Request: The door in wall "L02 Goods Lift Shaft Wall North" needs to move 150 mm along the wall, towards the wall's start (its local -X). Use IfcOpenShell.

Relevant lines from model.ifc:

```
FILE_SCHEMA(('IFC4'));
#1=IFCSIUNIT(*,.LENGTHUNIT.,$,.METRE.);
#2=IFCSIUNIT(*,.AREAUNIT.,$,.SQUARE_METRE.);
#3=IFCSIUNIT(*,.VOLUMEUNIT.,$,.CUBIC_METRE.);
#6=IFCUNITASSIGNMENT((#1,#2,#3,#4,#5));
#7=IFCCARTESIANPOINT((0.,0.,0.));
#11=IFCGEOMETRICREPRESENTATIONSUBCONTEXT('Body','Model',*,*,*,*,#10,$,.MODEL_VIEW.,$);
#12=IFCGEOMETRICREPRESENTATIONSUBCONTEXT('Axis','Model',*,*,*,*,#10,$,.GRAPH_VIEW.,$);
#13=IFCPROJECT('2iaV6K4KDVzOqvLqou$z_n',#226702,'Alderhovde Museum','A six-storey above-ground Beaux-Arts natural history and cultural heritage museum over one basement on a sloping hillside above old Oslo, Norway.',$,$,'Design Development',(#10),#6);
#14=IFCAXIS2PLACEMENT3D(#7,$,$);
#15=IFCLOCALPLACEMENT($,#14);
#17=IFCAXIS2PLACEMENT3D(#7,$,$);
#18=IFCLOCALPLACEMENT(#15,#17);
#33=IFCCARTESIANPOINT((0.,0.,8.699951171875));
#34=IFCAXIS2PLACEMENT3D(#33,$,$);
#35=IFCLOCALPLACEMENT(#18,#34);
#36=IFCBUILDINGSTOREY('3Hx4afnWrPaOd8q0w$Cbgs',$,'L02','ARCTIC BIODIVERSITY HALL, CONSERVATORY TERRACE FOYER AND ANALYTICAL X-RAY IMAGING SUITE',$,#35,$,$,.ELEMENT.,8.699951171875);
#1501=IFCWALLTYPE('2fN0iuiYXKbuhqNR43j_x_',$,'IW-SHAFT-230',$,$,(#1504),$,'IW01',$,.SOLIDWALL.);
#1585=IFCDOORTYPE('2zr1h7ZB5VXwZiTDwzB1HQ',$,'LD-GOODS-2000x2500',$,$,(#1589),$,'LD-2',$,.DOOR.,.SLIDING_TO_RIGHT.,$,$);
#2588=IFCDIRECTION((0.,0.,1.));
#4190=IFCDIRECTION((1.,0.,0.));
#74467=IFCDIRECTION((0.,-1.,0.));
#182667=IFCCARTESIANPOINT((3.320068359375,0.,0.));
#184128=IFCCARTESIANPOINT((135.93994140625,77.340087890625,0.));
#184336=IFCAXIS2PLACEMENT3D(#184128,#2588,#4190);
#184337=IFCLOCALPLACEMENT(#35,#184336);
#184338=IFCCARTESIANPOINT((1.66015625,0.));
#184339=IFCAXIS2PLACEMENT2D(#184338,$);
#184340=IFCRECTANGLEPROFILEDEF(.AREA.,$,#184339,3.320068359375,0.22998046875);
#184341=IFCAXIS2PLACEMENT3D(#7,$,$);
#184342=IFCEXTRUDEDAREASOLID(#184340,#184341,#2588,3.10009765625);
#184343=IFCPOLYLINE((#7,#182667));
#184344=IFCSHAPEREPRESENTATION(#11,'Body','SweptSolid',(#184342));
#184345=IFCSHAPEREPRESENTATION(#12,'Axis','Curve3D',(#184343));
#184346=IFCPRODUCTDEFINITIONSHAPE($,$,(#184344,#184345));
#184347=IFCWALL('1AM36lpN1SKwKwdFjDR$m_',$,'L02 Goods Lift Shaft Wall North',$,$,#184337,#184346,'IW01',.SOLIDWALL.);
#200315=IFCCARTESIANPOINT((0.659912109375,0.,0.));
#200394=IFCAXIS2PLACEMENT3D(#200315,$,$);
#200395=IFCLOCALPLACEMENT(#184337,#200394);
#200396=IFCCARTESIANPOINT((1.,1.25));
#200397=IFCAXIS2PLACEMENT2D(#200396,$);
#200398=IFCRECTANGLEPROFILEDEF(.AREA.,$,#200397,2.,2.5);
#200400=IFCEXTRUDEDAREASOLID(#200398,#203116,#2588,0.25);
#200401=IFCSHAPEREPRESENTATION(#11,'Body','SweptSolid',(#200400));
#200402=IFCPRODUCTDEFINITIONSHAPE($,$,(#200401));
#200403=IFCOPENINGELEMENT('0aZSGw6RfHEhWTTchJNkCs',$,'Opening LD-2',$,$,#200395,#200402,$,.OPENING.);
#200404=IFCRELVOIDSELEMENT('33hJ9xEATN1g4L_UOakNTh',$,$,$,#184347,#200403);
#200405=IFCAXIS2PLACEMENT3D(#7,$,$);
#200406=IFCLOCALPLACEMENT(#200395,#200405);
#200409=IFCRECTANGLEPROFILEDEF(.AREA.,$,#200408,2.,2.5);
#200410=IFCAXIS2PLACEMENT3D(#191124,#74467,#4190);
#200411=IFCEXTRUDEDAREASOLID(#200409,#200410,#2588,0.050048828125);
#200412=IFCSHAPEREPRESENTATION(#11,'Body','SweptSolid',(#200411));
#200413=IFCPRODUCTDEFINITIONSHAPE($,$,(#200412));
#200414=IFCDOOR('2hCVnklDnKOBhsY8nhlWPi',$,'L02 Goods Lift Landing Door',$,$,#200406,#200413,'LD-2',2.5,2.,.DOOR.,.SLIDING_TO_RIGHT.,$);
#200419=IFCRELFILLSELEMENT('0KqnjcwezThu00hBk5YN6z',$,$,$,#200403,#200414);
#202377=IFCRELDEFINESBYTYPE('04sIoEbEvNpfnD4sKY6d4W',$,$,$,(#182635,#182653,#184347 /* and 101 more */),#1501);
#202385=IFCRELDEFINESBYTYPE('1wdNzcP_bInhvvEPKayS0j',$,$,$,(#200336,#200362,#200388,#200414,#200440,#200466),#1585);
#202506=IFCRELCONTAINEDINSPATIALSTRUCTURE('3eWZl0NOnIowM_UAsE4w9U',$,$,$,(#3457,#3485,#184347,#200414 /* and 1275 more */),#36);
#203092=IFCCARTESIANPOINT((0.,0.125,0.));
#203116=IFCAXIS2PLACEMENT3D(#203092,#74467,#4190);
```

```python
import ifcopenshell
import ifcopenshell.api.geometry
import ifcopenshell.util.placement
import ifcopenshell.util.unit

model = ifcopenshell.open("model.ifc")
unit_scale = ifcopenshell.util.unit.calculate_unit_scale(model)

door = model.by_id(200414)
opening = door.FillsVoids[0].RelatingOpeningElement
wall = opening.VoidsElements[0].RelatingBuildingElement

wall_matrix = ifcopenshell.util.placement.get_local_placement(wall.ObjectPlacement)
shift = wall_matrix[:3, 0] * -0.15 / unit_scale
before = ifcopenshell.util.placement.get_local_placement(door.ObjectPlacement)[:3, 3].copy()

# The door is placed relative to its opening, so it follows when the opening moves.
matrix = ifcopenshell.util.placement.get_local_placement(opening.ObjectPlacement)
matrix[:3, 3] += shift
ifcopenshell.api.geometry.edit_object_placement(
    model, product=opening, matrix=matrix, is_si=False, should_transform_children=True
)

after = ifcopenshell.util.placement.get_local_placement(door.ObjectPlacement)[:3, 3]
print("door moved by", (after - before).round(3) + 0.0)

model.write("model_v2.ifc")
```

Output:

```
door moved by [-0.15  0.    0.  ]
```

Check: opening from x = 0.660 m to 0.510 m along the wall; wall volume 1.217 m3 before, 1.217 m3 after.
